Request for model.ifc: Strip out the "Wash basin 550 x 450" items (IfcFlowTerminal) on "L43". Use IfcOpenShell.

First a look at what the model holds.

```python
import ifcopenshell
import ifcopenshell.util.element

model = ifcopenshell.open("model.ifc")
print(model.schema)
storey = next(s for s in model.by_type("IfcBuildingStorey") if s.Name == "L43")
terminals = [e for e in ifcopenshell.util.element.get_decomposition(storey) if e.is_a("IfcFlowTerminal")]
seen = {}
for e in terminals:
    element_type = ifcopenshell.util.element.get_type(e)
    name = element_type.Name if element_type not in (None, e) else None
    seen[name] = seen.get(name, 0) + 1
for name, count in sorted(seen.items(), key=str):
    print(count, "x", name)
```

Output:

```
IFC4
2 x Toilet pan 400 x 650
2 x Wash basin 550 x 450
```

```python
import ifcopenshell
import ifcopenshell.api.root
import ifcopenshell.util.element

model = ifcopenshell.open("model.ifc")

storey = next(s for s in model.by_type("IfcBuildingStorey") if s.Name == "L43")
terminals = [e for e in ifcopenshell.util.element.get_decomposition(storey) if e.is_a("IfcFlowTerminal")]
targets = [e for e in terminals if (t := ifcopenshell.util.element.get_type(e)) not in (None, e) and t.Name == "Wash basin 550 x 450"]

for e in targets:
    ifcopenshell.api.root.remove_product(model, product=e)
print(len(targets), "removed")

model.write("model_updated.ifc")
```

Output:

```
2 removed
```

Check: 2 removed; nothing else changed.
